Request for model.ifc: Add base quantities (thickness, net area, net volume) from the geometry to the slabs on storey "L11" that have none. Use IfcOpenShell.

First a look at what the model holds.

```python
import ifcopenshell
import ifcopenshell.util.element
import ifcopenshell.util.unit

model = ifcopenshell.open("model.ifc")
print(model.schema)
for unit_type in ("LENGTHUNIT", "AREAUNIT", "VOLUMEUNIT"):
    print(unit_type, ifcopenshell.util.unit.calculate_unit_scale(model, unit_type))
storey = next(s for s in model.by_type("IfcBuildingStorey") if s.Name == "L11")
slabs = [e for e in ifcopenshell.util.element.get_decomposition(storey) if e.is_a("IfcSlab")]
for e in sorted(slabs, key=lambda e: e.id()):
    print(e.id(), e.is_a(), e.Name, list(ifcopenshell.util.element.get_psets(e, qtos_only=True)), sep=" | ")
```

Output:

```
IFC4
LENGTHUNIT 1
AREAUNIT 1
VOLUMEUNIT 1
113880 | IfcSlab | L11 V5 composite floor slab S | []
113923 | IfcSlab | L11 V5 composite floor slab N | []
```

```python
import ifcopenshell
import ifcopenshell.api.pset
import ifcopenshell.geom
import ifcopenshell.util.element
import ifcopenshell.util.shape
import ifcopenshell.util.unit

model = ifcopenshell.open("model.ifc")
unit_scale = ifcopenshell.util.unit.calculate_unit_scale(model)
area_scale = ifcopenshell.util.unit.calculate_unit_scale(model, "AREAUNIT")
volume_scale = ifcopenshell.util.unit.calculate_unit_scale(model, "VOLUMEUNIT")
settings = ifcopenshell.geom.settings()

storey = next(s for s in model.by_type("IfcBuildingStorey") if s.Name == "L11")
slabs = [e for e in ifcopenshell.util.element.get_decomposition(storey) if e.is_a("IfcSlab")]

for e in sorted(slabs, key=lambda e: e.id()):
    if ifcopenshell.util.element.get_psets(e, qtos_only=True, should_inherit=False):
        continue
    # Geometry comes back in metres, in the element's own axes.
    shape = ifcopenshell.geom.create_shape(settings, e)
    values = {
        "Width": ifcopenshell.util.shape.get_z(shape.geometry) / unit_scale,
        "NetArea": ifcopenshell.util.shape.get_footprint_area(shape.geometry) / area_scale,
        "NetVolume": ifcopenshell.util.shape.get_volume(shape.geometry) / volume_scale,
    }
    qto = ifcopenshell.api.pset.add_qto(model, product=e, name="Qto_SlabBaseQuantities")
    ifcopenshell.api.pset.edit_qto(model, qto=qto, properties=values)
    print(e.id(), {k: round(v, 3) for k, v in values.items()})

model.write("model_edited.ifc")
```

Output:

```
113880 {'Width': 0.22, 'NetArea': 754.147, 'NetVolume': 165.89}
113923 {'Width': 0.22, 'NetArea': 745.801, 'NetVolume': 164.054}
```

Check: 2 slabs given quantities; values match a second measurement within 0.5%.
